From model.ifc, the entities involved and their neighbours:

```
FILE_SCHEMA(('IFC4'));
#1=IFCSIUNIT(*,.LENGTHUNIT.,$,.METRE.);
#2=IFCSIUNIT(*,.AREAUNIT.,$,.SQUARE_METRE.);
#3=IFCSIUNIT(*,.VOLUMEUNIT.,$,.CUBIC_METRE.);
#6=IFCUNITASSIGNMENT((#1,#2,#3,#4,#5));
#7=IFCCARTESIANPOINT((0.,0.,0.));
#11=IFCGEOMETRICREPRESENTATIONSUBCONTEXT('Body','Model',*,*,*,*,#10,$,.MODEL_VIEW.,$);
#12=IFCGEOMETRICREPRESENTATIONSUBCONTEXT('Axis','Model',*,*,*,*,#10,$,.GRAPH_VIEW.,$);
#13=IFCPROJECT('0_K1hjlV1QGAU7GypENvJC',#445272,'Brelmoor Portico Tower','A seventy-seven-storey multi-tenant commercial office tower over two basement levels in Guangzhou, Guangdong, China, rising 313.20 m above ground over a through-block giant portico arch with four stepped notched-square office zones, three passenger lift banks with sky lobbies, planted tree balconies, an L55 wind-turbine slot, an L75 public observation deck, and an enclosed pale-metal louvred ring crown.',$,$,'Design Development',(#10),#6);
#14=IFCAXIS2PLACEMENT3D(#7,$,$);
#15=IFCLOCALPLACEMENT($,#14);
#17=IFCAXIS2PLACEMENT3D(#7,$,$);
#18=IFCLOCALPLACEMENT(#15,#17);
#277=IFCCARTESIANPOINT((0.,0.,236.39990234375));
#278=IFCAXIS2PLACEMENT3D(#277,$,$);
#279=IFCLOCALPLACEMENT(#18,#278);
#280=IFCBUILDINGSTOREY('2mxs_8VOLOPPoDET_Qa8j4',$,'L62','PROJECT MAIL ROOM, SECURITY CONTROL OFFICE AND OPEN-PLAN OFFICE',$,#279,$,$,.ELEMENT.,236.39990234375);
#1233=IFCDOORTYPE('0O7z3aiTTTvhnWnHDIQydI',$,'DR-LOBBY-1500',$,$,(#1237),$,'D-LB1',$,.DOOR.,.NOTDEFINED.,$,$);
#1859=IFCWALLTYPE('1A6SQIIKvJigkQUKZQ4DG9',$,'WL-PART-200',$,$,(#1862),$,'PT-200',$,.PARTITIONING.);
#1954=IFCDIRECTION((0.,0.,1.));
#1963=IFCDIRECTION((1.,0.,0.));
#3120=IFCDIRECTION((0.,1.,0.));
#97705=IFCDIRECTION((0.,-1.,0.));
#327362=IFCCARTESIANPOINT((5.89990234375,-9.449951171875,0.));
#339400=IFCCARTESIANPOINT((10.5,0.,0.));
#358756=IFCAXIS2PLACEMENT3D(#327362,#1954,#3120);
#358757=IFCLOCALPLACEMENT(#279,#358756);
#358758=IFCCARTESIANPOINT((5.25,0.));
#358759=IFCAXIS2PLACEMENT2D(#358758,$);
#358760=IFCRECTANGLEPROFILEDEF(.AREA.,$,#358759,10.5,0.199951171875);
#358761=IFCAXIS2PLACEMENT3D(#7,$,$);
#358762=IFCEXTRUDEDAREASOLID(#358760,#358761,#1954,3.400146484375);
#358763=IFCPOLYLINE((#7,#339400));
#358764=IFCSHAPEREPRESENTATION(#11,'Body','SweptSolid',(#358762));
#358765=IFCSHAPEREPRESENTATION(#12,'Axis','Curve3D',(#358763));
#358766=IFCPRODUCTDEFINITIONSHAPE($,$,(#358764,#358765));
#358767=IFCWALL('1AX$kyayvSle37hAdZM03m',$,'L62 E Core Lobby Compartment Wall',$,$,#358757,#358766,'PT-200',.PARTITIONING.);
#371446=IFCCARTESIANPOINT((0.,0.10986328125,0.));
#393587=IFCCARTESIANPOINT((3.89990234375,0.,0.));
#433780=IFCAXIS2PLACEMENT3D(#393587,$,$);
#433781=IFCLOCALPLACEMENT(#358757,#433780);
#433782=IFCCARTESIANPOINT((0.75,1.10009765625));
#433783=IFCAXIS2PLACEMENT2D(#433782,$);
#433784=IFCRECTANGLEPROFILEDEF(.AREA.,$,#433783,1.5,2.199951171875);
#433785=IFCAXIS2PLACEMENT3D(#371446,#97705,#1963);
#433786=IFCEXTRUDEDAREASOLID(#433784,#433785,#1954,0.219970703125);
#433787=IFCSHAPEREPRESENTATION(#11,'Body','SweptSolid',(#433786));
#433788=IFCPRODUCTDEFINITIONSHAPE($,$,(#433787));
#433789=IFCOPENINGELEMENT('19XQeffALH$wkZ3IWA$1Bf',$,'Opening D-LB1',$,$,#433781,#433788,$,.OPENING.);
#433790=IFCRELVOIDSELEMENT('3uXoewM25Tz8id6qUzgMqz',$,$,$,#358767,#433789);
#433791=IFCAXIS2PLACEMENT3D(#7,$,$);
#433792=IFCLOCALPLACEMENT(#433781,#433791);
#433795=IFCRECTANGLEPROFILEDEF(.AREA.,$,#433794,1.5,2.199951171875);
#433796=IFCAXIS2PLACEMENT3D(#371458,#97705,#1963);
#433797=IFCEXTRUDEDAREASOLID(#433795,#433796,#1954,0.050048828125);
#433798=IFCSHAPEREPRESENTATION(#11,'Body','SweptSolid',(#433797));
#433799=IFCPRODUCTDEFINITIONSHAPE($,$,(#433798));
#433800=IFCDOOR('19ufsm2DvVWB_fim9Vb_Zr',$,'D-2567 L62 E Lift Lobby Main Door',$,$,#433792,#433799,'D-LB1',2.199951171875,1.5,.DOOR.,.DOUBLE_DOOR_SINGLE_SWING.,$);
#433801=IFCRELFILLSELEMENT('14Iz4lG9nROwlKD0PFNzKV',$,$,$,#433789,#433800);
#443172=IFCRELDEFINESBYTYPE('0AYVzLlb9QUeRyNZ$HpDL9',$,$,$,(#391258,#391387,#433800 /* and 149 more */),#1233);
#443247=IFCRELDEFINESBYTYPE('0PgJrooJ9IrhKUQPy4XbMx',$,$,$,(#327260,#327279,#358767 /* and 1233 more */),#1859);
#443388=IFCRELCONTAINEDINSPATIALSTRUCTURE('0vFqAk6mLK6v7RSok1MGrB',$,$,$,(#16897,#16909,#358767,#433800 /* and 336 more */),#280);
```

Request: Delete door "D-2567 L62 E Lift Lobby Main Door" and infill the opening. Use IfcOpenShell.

```python
import ifcopenshell
import ifcopenshell.api.feature
import ifcopenshell.api.root
import ifcopenshell.geom
import ifcopenshell.util.shape

model = ifcopenshell.open("model.ifc")
settings = ifcopenshell.geom.settings()


def volume(element):
    """Net volume in cubic metres, openings subtracted."""
    shape = ifcopenshell.geom.create_shape(settings, element)
    return ifcopenshell.util.shape.get_volume(shape.geometry)


door = model.by_guid("19ufsm2DvVWB_fim9Vb_Zr")
opening = door.FillsVoids[0].RelatingOpeningElement
wall = opening.VoidsElements[0].RelatingBuildingElement
before = volume(wall)

ifcopenshell.api.root.remove_product(model, product=door)
ifcopenshell.api.feature.remove_feature(model, feature=opening)

after = volume(wall)

print(f"wall volume {before:.3f} -> {after:.3f} m3")

model.write("model_edited.ifc")
```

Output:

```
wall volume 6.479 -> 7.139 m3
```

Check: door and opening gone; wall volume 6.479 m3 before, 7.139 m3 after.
